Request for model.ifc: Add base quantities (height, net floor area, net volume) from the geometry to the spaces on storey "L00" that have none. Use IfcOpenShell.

First a look at what the model holds.

```python
import ifcopenshell
import ifcopenshell.util.element
import ifcopenshell.util.unit

model = ifcopenshell.open("model.ifc")
print(model.schema)
for unit_type in ("LENGTHUNIT", "AREAUNIT", "VOLUMEUNIT"):
    print(unit_type, ifcopenshell.util.unit.calculate_unit_scale(model, unit_type))
storey = next(s for s in model.by_type("IfcBuildingStorey") if s.Name == "L00")
spaces = [e for e in ifcopenshell.util.element.get_decomposition(storey) if e.is_a("IfcSpace")]
for e in sorted(spaces, key=lambda e: e.id()):
    print(e.id(), e.is_a(), e.Name, list(ifcopenshell.util.element.get_psets(e, qtos_only=True)), sep=" | ")
```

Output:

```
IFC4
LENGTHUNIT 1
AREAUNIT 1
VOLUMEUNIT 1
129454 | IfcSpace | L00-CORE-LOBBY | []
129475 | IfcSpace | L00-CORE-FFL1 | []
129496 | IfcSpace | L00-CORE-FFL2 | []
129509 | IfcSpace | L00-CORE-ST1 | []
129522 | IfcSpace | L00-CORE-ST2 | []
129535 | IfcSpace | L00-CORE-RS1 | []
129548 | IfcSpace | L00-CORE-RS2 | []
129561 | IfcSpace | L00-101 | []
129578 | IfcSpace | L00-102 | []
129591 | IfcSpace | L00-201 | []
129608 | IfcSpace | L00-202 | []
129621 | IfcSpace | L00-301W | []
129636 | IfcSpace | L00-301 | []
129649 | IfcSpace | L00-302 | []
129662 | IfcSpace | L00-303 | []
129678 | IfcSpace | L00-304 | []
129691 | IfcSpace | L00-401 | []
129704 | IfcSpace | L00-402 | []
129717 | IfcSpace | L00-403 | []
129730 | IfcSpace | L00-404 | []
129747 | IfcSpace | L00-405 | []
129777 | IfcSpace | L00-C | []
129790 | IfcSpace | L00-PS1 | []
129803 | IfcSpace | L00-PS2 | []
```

```python
import ifcopenshell
import ifcopenshell.api.pset
import ifcopenshell.geom
import ifcopenshell.util.element
import ifcopenshell.util.shape
import ifcopenshell.util.unit

model = ifcopenshell.open("model.ifc")
unit_scale = ifcopenshell.util.unit.calculate_unit_scale(model)
area_scale = ifcopenshell.util.unit.calculate_unit_scale(model, "AREAUNIT")
volume_scale = ifcopenshell.util.unit.calculate_unit_scale(model, "VOLUMEUNIT")
settings = ifcopenshell.geom.settings()

storey = next(s for s in model.by_type("IfcBuildingStorey") if s.Name == "L00")
spaces = [e for e in ifcopenshell.util.element.get_decomposition(storey) if e.is_a("IfcSpace")]

for e in sorted(spaces, key=lambda e: e.id()):
    if ifcopenshell.util.element.get_psets(e, qtos_only=True, should_inherit=False):
        continue
    # Geometry comes back in metres, in the element's own axes.
    shape = ifcopenshell.geom.create_shape(settings, e)
    values = {
        "Height": ifcopenshell.util.shape.get_z(shape.geometry) / unit_scale,
        "NetFloorArea": ifcopenshell.util.shape.get_footprint_area(shape.geometry) / area_scale,
        "NetVolume": ifcopenshell.util.shape.get_volume(shape.geometry) / volume_scale,
    }
    qto = ifcopenshell.api.pset.add_qto(model, product=e, name="Qto_SpaceBaseQuantities")
    ifcopenshell.api.pset.edit_qto(model, qto=qto, properties=values)
    print(e.id(), {k: round(v, 3) for k, v in values.items()})

model.write("model_edited.ifc")
```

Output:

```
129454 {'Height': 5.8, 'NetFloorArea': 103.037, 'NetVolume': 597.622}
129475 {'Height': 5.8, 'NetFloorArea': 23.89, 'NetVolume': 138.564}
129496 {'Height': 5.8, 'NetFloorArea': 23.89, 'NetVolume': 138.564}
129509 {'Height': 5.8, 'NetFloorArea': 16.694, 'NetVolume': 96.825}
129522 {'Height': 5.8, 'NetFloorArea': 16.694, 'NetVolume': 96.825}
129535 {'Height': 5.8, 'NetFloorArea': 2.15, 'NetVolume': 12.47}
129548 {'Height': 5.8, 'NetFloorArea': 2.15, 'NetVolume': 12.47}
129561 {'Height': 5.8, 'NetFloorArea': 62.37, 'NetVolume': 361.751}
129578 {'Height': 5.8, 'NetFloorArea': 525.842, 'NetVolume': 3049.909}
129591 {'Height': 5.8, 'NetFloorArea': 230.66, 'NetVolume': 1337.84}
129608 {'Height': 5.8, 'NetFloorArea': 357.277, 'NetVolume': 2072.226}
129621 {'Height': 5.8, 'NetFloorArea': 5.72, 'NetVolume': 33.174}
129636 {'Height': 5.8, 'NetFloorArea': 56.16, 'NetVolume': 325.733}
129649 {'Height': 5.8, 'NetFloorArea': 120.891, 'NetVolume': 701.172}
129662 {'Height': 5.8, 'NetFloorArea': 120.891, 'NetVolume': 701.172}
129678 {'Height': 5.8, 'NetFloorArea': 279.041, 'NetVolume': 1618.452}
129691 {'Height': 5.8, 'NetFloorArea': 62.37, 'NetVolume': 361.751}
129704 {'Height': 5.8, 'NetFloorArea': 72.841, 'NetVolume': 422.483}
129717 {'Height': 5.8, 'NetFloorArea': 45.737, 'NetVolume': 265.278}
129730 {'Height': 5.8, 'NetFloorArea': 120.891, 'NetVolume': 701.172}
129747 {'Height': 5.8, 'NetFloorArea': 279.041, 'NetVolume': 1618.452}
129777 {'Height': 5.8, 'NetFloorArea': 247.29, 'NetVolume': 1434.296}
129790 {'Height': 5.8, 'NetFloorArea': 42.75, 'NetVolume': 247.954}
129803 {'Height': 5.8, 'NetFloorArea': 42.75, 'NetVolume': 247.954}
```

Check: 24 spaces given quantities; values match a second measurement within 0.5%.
